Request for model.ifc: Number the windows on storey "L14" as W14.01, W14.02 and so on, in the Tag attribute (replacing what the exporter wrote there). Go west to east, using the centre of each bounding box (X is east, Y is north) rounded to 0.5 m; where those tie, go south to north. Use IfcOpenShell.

First a look at what the model holds.

```python
import ifcopenshell
import ifcopenshell.util.element
import ifcopenshell.util.placement

model = ifcopenshell.open("model.ifc")
print(model.schema)
storey = next(s for s in model.by_type("IfcBuildingStorey") if s.Name == "L14")
windows = [e for e in ifcopenshell.util.element.get_decomposition(storey) if e.is_a("IfcWindow")]
for e in sorted(windows, key=lambda e: e.id()):
    origin = ifcopenshell.util.placement.get_local_placement(e.ObjectPlacement)[:3, 3]
    print(e.id(), e.Tag, e.Name, origin.round(2) + 0.0, sep=" | ")
```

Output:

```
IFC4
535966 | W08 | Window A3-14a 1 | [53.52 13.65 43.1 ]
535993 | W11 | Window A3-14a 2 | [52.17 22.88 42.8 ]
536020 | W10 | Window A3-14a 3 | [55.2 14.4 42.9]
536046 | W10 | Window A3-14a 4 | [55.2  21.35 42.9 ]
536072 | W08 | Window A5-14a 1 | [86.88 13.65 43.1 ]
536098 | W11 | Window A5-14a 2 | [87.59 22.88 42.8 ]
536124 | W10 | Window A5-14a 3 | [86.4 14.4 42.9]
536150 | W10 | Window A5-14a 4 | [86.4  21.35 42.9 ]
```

```python
import ifcopenshell
import ifcopenshell.geom
import ifcopenshell.util.element
import ifcopenshell.util.shape

model = ifcopenshell.open("model.ifc")
settings = ifcopenshell.geom.settings()
settings.set("use-world-coords", True)


def centre(element):
    shape = ifcopenshell.geom.create_shape(settings, element)
    return ifcopenshell.util.shape.get_bbox_centroid(shape.geometry)


storey = next(s for s in model.by_type("IfcBuildingStorey") if s.Name == "L14")
windows = [e for e in ifcopenshell.util.element.get_decomposition(storey) if e.is_a("IfcWindow")]

# Insertion points can sit at a corner or the storey origin, so sort by the geometry (in metres).
centres = {e: centre(e) for e in windows}
windows.sort(key=lambda e: (round(centres[e][0] / 0.5), centres[e][1]))

for i, e in enumerate(windows, start=1):
    number = f"W14.{i:02d}"
    e.Tag = number
    print(e.id(), number)

model.write("model_edited.ifc")
```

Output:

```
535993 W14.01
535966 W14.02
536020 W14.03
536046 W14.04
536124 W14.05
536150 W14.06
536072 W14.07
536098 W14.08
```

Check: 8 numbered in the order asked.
